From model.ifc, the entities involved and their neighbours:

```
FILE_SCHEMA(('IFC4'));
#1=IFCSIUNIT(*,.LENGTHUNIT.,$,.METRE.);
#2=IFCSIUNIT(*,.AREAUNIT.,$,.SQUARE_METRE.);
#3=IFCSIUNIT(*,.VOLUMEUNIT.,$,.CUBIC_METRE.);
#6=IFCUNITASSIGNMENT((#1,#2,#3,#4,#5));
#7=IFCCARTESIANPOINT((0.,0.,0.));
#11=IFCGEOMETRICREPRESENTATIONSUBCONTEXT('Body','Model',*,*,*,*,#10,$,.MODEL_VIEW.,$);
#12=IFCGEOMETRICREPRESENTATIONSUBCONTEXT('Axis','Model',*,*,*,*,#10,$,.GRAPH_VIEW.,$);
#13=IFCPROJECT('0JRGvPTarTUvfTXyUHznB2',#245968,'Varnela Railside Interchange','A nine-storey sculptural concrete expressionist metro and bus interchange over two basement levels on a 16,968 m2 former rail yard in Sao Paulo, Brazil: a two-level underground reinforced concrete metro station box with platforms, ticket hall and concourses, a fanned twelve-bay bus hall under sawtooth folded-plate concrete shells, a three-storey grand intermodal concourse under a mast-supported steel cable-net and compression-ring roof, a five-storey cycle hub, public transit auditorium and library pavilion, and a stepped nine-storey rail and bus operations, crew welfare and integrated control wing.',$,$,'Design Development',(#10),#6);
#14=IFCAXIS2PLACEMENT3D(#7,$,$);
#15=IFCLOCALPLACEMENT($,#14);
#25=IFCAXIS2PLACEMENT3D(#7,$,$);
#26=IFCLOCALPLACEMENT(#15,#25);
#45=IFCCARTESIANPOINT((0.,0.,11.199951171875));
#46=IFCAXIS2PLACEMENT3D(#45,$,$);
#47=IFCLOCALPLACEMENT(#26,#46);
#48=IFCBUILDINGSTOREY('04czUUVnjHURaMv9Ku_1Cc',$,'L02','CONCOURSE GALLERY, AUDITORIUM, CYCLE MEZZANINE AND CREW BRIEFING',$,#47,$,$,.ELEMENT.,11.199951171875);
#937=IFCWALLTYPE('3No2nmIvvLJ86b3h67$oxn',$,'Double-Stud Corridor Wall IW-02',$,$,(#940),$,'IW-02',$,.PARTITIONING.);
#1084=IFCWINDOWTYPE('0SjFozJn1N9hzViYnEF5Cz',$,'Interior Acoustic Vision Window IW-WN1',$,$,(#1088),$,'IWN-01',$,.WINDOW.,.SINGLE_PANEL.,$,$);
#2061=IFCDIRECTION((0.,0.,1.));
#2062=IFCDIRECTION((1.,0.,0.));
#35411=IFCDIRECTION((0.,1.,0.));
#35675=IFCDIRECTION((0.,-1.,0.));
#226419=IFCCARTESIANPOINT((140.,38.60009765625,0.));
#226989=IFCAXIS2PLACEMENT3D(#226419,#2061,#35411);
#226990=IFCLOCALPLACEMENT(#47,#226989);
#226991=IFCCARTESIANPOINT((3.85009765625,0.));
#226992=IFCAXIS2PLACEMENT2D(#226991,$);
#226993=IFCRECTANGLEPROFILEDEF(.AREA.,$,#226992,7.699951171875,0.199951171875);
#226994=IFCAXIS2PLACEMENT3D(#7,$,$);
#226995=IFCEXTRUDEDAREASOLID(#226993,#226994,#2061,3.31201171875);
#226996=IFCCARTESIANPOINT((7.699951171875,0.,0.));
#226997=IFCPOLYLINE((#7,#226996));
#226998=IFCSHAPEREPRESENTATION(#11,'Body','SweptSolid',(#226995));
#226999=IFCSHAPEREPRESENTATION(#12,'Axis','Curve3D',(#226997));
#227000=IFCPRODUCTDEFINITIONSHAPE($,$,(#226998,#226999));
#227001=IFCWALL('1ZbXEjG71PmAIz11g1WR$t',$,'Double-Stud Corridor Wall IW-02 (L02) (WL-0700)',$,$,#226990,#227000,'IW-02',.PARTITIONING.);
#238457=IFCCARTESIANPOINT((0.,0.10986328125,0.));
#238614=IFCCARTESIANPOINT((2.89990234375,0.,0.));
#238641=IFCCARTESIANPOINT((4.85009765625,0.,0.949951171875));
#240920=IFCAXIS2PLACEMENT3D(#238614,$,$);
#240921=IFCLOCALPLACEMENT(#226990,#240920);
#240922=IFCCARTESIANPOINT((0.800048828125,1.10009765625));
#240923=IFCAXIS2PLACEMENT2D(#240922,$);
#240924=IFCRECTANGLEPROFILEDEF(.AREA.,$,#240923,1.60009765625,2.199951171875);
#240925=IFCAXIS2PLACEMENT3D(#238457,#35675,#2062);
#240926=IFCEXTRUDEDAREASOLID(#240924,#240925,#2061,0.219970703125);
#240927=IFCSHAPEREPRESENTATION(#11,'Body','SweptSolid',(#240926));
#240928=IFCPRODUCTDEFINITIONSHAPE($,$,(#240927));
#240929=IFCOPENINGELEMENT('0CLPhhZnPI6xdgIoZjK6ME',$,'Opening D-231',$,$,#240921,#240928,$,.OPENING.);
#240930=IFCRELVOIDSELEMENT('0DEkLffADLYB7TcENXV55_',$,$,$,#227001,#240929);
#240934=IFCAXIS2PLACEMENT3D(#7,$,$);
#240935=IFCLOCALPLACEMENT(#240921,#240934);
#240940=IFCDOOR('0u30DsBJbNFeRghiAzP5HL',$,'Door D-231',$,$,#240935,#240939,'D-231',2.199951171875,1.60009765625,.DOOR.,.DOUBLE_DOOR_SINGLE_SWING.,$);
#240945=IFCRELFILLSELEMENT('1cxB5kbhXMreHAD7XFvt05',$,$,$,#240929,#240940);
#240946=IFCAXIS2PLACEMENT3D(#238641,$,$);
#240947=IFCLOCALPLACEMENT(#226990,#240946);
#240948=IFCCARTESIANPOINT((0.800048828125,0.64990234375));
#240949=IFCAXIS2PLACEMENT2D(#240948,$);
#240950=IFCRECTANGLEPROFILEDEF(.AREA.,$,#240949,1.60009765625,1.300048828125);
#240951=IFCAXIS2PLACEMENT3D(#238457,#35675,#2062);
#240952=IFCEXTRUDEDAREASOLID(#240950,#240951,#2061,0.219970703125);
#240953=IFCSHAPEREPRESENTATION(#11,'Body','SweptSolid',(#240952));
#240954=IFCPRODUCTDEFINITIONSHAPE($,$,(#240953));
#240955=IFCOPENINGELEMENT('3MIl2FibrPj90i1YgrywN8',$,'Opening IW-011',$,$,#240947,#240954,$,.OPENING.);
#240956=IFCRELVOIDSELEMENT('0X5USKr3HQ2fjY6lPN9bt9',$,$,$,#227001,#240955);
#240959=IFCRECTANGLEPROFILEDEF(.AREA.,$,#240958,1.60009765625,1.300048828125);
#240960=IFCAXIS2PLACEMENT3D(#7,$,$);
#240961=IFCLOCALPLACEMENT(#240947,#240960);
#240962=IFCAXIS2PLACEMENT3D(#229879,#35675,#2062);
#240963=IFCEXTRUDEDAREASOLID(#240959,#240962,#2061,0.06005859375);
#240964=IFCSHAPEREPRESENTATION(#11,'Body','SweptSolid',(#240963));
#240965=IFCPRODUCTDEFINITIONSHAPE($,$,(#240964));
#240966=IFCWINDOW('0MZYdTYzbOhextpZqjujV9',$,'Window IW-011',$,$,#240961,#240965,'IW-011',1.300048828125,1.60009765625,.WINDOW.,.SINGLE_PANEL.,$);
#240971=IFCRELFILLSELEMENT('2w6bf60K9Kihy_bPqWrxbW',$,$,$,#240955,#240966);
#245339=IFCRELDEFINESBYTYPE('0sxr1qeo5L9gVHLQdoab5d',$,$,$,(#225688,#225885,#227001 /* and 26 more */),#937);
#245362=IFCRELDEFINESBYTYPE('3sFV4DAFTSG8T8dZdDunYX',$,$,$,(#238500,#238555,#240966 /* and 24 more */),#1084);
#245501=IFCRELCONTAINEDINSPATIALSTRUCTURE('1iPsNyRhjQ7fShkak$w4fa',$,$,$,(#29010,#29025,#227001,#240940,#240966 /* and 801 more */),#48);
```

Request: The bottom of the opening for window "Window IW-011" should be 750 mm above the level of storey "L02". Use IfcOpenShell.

```python
import numpy as np
import ifcopenshell
import ifcopenshell.api.geometry
import ifcopenshell.geom
import ifcopenshell.util.element
import ifcopenshell.util.placement
import ifcopenshell.util.shape
import ifcopenshell.util.unit

model = ifcopenshell.open("model.ifc")
unit_scale = ifcopenshell.util.unit.calculate_unit_scale(model)

window = model.by_id(240966)
opening = window.FillsVoids[0].RelatingOpeningElement
storey = ifcopenshell.util.element.get_container(window, ifc_class="IfcBuildingStorey")
level = ifcopenshell.util.placement.get_local_placement(storey.ObjectPlacement)[2, 3]

# The opening's origin need not be at the sill, so measure its lowest point.
shape = ifcopenshell.geom.create_shape(ifcopenshell.geom.settings(), opening)
bottom = ifcopenshell.util.shape.get_shape_bottom_elevation(shape, shape.geometry) / unit_scale
dz = level + 0.75 / unit_scale - bottom

shift = np.array([0.0, 0.0, dz])
# The window is placed relative to its opening, so it follows when the opening moves.
matrix = ifcopenshell.util.placement.get_local_placement(opening.ObjectPlacement)
matrix[:3, 3] += shift
ifcopenshell.api.geometry.edit_object_placement(
    model, product=opening, matrix=matrix, is_si=False, should_transform_children=True
)

print(f"moved by {dz * unit_scale:+.3f} m")

model.write("model-out.ifc")
```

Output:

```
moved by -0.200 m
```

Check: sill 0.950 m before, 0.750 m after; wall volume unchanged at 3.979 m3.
